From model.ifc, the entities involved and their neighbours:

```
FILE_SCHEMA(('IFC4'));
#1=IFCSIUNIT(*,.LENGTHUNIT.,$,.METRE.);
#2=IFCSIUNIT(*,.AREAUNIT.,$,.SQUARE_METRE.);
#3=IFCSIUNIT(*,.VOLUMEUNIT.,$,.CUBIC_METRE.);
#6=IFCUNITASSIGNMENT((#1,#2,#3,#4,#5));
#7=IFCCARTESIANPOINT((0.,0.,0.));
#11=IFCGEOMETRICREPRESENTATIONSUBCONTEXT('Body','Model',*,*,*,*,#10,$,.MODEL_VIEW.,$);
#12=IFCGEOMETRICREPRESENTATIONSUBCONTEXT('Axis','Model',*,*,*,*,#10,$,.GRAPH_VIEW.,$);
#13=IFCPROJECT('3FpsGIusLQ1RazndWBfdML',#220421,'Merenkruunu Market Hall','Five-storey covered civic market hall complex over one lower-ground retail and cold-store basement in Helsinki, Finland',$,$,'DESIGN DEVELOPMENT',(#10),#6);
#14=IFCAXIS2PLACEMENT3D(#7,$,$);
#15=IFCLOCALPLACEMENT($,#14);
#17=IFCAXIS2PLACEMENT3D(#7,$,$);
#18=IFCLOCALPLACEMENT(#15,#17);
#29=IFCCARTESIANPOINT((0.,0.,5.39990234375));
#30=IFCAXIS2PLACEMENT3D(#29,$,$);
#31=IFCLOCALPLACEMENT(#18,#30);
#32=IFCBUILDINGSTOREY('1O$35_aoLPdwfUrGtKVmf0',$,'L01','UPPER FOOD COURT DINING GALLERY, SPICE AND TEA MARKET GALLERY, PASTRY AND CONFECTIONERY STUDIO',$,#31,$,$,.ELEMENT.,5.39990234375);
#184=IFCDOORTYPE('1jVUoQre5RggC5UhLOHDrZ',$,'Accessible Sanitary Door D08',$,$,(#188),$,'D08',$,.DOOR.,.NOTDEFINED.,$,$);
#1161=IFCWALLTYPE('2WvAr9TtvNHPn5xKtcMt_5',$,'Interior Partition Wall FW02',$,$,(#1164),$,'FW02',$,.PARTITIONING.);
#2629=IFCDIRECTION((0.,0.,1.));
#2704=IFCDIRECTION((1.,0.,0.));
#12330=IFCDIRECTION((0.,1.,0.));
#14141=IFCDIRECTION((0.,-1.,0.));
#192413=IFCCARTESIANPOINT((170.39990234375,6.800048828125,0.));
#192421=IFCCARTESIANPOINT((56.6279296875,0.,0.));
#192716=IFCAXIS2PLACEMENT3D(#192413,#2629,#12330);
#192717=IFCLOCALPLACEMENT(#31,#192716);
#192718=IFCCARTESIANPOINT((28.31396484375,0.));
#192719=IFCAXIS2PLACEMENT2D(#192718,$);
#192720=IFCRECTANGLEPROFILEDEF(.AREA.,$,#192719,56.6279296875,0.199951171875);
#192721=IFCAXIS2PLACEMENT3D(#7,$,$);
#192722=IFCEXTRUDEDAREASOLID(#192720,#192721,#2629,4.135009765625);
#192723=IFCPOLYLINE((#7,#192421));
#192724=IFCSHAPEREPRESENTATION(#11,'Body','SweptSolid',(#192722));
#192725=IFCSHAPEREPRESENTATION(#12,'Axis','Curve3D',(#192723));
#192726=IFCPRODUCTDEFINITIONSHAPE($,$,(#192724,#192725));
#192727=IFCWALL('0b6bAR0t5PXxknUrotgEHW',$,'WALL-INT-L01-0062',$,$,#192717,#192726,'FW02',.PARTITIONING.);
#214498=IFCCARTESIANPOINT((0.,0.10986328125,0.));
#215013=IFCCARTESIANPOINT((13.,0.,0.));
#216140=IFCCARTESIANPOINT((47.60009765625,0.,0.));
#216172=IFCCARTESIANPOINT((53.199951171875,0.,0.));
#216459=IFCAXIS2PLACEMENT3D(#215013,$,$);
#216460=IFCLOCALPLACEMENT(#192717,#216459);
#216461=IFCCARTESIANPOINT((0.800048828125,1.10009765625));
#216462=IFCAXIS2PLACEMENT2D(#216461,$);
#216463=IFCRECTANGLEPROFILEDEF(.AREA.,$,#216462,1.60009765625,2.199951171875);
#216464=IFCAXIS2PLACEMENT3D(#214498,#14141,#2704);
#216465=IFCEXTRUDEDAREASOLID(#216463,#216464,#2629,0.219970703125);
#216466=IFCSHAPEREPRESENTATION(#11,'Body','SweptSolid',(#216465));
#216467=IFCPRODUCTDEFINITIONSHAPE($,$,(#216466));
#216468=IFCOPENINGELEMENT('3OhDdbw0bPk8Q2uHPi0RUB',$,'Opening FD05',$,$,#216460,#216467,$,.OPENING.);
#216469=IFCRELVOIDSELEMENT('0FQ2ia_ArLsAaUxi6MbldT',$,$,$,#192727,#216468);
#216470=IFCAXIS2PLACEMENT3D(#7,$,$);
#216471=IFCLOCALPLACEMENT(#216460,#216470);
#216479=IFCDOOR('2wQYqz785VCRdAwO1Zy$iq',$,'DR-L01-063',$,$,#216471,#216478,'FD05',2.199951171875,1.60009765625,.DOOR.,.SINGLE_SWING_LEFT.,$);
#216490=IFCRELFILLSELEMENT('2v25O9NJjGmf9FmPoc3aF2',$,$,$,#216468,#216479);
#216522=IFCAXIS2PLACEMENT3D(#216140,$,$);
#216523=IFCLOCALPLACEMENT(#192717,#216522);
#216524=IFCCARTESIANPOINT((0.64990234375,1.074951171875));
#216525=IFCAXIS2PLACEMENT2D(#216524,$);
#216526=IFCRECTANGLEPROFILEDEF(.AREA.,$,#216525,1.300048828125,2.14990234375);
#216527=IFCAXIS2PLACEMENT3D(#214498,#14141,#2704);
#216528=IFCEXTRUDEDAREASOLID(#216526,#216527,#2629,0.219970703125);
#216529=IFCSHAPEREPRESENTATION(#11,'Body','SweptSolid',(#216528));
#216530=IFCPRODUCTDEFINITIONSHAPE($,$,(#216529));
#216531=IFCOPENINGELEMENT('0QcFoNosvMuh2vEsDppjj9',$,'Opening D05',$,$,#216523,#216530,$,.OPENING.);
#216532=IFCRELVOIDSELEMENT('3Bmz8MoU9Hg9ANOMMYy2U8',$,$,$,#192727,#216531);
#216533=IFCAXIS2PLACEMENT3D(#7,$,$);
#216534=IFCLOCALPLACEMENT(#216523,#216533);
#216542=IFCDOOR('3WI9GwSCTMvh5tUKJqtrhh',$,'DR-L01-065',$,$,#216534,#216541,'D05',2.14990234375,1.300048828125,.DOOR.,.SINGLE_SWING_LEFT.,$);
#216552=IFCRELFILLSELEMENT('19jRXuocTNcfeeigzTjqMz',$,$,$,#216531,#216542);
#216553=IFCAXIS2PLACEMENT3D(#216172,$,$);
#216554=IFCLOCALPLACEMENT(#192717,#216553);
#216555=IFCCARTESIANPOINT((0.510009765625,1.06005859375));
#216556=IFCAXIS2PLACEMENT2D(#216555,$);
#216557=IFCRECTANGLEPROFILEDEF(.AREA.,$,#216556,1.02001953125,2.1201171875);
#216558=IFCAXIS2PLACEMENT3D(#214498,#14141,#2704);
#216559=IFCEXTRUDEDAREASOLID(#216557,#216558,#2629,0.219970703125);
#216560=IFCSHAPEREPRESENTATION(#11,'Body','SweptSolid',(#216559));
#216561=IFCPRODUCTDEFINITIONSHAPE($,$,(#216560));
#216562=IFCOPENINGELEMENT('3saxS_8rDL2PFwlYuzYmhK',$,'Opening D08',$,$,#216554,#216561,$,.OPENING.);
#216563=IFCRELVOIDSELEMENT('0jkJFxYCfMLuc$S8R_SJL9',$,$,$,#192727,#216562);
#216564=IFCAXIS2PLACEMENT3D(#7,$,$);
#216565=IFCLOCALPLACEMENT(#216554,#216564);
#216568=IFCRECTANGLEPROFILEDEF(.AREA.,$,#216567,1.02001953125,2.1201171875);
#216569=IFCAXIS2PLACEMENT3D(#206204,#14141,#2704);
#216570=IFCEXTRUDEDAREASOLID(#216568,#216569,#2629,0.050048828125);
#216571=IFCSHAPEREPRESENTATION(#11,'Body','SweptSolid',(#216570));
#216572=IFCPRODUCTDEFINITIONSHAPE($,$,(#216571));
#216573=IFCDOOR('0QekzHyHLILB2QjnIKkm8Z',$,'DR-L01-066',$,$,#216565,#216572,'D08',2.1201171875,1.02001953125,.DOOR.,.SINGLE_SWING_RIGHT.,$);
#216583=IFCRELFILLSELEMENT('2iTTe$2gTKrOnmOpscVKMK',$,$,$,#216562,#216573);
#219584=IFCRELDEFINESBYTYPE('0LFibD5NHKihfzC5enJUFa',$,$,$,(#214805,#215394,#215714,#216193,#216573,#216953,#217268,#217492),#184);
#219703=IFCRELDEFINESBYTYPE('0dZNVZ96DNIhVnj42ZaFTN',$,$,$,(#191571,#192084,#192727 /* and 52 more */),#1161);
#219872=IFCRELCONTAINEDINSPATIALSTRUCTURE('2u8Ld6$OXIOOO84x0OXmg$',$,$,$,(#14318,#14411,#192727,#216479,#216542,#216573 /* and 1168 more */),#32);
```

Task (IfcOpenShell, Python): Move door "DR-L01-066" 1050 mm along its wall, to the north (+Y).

```python
import ifcopenshell
import ifcopenshell.api.geometry
import ifcopenshell.util.placement
import ifcopenshell.util.unit

model = ifcopenshell.open("model.ifc")
unit_scale = ifcopenshell.util.unit.calculate_unit_scale(model)

door = model.by_guid("0QekzHyHLILB2QjnIKkm8Z")
opening = door.FillsVoids[0].RelatingOpeningElement
wall = opening.VoidsElements[0].RelatingBuildingElement

wall_matrix = ifcopenshell.util.placement.get_local_placement(wall.ObjectPlacement)
shift = wall_matrix[:3, 0] * 1.05 / unit_scale
before = ifcopenshell.util.placement.get_local_placement(door.ObjectPlacement)[:3, 3].copy()

# The door is placed relative to its opening, so it follows when the opening moves.
matrix = ifcopenshell.util.placement.get_local_placement(opening.ObjectPlacement)
matrix[:3, 3] += shift
ifcopenshell.api.geometry.edit_object_placement(
    model, product=opening, matrix=matrix, is_si=False, should_transform_children=True
)

after = ifcopenshell.util.placement.get_local_placement(door.ObjectPlacement)[:3, 3]
print("door moved by", (after - before).round(3) + 0.0)

model.write("model_rev.ifc")
```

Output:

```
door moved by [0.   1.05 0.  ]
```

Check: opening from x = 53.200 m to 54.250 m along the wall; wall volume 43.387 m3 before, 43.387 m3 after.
